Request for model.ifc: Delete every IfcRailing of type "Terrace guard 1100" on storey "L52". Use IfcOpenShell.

First a look at what the model holds.

```python
import ifcopenshell
import ifcopenshell.util.element

model = ifcopenshell.open("model.ifc")
print(model.schema)
storey = next(s for s in model.by_type("IfcBuildingStorey") if s.Name == "L52")
railings = [e for e in ifcopenshell.util.element.get_decomposition(storey) if e.is_a("IfcRailing")]
seen = {}
for e in railings:
    element_type = ifcopenshell.util.element.get_type(e)
    name = element_type.Name if element_type not in (None, e) else None
    seen[name] = seen.get(name, 0) + 1
for name, count in sorted(seen.items(), key=str):
    print(count, "x", name)
```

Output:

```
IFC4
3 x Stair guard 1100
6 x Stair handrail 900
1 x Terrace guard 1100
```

```python
import ifcopenshell
import ifcopenshell.api.root
import ifcopenshell.util.element

model = ifcopenshell.open("model.ifc")

storey = next(s for s in model.by_type("IfcBuildingStorey") if s.Name == "L52")
railings = [e for e in ifcopenshell.util.element.get_decomposition(storey) if e.is_a("IfcRailing")]
targets = [e for e in railings if (t := ifcopenshell.util.element.get_type(e)) not in (None, e) and t.Name == "Terrace guard 1100"]

for e in targets:
    ifcopenshell.api.root.remove_product(model, product=e)
print(len(targets), "removed")

model.write("model_v2.ifc")
```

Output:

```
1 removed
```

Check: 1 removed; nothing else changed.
